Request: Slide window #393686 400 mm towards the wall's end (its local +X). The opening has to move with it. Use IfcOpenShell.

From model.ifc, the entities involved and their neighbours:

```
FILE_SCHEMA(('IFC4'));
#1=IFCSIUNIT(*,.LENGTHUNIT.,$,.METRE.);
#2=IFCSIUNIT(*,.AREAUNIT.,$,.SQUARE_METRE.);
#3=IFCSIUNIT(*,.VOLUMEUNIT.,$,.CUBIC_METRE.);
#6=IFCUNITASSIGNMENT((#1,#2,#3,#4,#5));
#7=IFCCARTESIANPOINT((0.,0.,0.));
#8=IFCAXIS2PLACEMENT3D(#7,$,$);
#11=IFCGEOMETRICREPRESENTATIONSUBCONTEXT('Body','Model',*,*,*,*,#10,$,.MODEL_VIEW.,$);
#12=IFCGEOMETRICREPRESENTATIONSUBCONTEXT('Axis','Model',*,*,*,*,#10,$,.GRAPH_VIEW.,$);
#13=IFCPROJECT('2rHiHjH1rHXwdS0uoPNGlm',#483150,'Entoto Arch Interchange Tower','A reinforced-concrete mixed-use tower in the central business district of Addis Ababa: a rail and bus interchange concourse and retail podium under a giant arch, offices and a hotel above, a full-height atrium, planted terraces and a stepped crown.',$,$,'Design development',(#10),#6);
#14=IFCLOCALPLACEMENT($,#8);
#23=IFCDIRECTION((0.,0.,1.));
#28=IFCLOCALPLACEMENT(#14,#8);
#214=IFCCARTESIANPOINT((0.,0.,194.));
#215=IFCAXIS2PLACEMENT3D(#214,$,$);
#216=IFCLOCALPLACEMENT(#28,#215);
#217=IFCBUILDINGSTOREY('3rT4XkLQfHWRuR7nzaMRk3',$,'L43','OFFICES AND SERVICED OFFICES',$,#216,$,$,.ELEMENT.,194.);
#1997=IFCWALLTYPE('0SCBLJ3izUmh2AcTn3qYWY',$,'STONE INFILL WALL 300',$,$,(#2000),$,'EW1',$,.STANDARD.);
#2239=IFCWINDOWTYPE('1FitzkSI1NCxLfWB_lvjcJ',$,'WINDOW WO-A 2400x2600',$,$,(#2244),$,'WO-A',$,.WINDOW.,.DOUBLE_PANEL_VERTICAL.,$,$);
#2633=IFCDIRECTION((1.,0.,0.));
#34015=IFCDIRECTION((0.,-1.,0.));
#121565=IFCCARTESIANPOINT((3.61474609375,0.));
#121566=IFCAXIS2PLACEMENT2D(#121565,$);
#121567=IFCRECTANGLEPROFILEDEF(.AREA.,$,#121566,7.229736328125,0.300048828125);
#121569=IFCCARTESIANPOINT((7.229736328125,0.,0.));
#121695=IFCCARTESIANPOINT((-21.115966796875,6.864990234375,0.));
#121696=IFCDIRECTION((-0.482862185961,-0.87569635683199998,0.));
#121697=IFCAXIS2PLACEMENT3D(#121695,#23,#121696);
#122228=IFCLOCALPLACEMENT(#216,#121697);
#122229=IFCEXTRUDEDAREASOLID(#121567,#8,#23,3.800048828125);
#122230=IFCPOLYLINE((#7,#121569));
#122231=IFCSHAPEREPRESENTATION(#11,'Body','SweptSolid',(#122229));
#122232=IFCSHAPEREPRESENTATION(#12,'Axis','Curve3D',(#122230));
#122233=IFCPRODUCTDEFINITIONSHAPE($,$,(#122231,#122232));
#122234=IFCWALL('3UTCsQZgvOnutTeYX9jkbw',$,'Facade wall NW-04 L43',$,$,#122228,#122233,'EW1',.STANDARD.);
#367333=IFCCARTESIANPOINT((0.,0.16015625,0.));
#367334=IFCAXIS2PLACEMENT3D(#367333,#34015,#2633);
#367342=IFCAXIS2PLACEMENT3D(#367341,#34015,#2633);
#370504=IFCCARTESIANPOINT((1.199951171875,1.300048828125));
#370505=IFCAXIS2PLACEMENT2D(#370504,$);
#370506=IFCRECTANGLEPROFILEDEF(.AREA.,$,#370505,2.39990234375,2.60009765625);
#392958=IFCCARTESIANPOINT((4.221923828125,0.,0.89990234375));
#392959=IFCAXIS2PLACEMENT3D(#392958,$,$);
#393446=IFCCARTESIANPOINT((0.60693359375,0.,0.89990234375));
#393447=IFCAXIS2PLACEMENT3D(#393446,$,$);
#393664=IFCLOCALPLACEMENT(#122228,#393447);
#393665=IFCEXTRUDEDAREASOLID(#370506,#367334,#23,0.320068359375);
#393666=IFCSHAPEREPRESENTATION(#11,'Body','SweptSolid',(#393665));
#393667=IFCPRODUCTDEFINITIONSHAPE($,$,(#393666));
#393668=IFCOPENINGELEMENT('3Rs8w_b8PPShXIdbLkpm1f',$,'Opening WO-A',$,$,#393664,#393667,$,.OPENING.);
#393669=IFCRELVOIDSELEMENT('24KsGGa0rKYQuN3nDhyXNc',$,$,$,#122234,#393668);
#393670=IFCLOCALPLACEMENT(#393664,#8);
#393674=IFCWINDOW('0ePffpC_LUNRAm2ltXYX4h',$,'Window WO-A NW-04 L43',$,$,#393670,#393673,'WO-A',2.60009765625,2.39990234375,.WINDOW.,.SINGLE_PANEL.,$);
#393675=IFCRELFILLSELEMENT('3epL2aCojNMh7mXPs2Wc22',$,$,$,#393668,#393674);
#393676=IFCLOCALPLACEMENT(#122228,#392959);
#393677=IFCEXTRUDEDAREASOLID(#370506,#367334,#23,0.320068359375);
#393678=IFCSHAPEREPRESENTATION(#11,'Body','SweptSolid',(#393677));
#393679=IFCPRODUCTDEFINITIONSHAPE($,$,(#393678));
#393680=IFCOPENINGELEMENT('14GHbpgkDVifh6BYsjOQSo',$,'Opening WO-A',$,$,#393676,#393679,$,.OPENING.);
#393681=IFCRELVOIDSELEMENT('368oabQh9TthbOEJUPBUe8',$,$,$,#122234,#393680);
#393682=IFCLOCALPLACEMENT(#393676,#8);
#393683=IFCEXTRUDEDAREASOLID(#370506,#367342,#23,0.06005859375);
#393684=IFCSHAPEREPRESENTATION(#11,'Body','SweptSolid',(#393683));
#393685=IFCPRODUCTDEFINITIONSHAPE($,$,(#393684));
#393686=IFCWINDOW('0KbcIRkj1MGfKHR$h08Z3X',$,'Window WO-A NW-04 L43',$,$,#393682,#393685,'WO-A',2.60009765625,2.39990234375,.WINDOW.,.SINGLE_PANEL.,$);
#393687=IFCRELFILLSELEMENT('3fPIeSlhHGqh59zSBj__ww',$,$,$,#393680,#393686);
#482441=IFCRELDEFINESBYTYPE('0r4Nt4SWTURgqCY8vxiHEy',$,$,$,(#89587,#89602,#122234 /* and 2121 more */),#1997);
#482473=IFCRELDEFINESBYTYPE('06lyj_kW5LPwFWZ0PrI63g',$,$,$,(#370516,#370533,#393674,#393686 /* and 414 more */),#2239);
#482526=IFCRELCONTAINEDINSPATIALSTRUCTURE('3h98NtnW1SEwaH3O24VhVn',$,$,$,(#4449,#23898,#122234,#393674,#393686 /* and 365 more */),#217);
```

```python
import ifcopenshell
import ifcopenshell.api.geometry
import ifcopenshell.util.placement
import ifcopenshell.util.unit

model = ifcopenshell.open("model.ifc")
unit_scale = ifcopenshell.util.unit.calculate_unit_scale(model)

window = model.by_guid("0KbcIRkj1MGfKHR$h08Z3X")
opening = window.FillsVoids[0].RelatingOpeningElement
wall = opening.VoidsElements[0].RelatingBuildingElement

wall_matrix = ifcopenshell.util.placement.get_local_placement(wall.ObjectPlacement)
shift = wall_matrix[:3, 0] * 0.4 / unit_scale
before = ifcopenshell.util.placement.get_local_placement(window.ObjectPlacement)[:3, 3].copy()

# The window is placed relative to its opening, so it follows when the opening moves.
matrix = ifcopenshell.util.placement.get_local_placement(opening.ObjectPlacement)
matrix[:3, 3] += shift
ifcopenshell.api.geometry.edit_object_placement(
    model, product=opening, matrix=matrix, is_si=False, should_transform_children=True
)

after = ifcopenshell.util.placement.get_local_placement(window.ObjectPlacement)[:3, 3]
print("window moved by", (after - before).round(3) + 0.0)

model.write("model_edited.ifc")
```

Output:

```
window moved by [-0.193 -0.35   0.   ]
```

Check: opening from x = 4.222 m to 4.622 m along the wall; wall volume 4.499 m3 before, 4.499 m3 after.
